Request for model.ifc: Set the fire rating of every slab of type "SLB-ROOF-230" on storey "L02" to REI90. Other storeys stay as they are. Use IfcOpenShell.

First a look at what the model holds.

```python
import ifcopenshell
import ifcopenshell.util.element

model = ifcopenshell.open("model.ifc")
print(model.schema)
storey = next(s for s in model.by_type("IfcBuildingStorey") if s.Name == "L02")
slabs = [e for e in ifcopenshell.util.element.get_decomposition(storey) if e.is_a("IfcSlab")]
seen = {}
for e in slabs:
    element_type = ifcopenshell.util.element.get_type(e)
    key = (element_type.Name if element_type != e and element_type else None, ifcopenshell.util.element.get_pset(e, "Pset_SlabCommon", "FireRating"))
    seen[key] = seen.get(key, 0) + 1
for (name, value), count in sorted(seen.items(), key=str):
    print(count, "x", name, "|", value)
```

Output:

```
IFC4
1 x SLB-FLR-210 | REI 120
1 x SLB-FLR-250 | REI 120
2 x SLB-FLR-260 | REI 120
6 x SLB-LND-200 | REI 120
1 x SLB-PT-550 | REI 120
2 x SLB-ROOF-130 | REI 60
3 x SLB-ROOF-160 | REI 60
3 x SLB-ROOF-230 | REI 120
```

```python
import ifcopenshell
import ifcopenshell.api.pset
import ifcopenshell.util.element

model = ifcopenshell.open("model.ifc")

storey = next(s for s in model.by_type("IfcBuildingStorey") if s.Name == "L02")
slabs = [e for e in ifcopenshell.util.element.get_decomposition(storey) if e.is_a("IfcSlab")]

count = 0
for e in slabs:
    element_type = ifcopenshell.util.element.get_type(e)
    if element_type in (None, e) or element_type.Name != "SLB-ROOF-230":
        continue
    # add_pset returns the element's existing set when there is one.
    pset = ifcopenshell.api.pset.add_pset(model, product=e, name="Pset_SlabCommon")
    ifcopenshell.api.pset.edit_pset(model, pset=pset, properties={"FireRating": "REI90"})
    count += 1

print(count, "slabs updated")

model.write("model_edited.ifc")
```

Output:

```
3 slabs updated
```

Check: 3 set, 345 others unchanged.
